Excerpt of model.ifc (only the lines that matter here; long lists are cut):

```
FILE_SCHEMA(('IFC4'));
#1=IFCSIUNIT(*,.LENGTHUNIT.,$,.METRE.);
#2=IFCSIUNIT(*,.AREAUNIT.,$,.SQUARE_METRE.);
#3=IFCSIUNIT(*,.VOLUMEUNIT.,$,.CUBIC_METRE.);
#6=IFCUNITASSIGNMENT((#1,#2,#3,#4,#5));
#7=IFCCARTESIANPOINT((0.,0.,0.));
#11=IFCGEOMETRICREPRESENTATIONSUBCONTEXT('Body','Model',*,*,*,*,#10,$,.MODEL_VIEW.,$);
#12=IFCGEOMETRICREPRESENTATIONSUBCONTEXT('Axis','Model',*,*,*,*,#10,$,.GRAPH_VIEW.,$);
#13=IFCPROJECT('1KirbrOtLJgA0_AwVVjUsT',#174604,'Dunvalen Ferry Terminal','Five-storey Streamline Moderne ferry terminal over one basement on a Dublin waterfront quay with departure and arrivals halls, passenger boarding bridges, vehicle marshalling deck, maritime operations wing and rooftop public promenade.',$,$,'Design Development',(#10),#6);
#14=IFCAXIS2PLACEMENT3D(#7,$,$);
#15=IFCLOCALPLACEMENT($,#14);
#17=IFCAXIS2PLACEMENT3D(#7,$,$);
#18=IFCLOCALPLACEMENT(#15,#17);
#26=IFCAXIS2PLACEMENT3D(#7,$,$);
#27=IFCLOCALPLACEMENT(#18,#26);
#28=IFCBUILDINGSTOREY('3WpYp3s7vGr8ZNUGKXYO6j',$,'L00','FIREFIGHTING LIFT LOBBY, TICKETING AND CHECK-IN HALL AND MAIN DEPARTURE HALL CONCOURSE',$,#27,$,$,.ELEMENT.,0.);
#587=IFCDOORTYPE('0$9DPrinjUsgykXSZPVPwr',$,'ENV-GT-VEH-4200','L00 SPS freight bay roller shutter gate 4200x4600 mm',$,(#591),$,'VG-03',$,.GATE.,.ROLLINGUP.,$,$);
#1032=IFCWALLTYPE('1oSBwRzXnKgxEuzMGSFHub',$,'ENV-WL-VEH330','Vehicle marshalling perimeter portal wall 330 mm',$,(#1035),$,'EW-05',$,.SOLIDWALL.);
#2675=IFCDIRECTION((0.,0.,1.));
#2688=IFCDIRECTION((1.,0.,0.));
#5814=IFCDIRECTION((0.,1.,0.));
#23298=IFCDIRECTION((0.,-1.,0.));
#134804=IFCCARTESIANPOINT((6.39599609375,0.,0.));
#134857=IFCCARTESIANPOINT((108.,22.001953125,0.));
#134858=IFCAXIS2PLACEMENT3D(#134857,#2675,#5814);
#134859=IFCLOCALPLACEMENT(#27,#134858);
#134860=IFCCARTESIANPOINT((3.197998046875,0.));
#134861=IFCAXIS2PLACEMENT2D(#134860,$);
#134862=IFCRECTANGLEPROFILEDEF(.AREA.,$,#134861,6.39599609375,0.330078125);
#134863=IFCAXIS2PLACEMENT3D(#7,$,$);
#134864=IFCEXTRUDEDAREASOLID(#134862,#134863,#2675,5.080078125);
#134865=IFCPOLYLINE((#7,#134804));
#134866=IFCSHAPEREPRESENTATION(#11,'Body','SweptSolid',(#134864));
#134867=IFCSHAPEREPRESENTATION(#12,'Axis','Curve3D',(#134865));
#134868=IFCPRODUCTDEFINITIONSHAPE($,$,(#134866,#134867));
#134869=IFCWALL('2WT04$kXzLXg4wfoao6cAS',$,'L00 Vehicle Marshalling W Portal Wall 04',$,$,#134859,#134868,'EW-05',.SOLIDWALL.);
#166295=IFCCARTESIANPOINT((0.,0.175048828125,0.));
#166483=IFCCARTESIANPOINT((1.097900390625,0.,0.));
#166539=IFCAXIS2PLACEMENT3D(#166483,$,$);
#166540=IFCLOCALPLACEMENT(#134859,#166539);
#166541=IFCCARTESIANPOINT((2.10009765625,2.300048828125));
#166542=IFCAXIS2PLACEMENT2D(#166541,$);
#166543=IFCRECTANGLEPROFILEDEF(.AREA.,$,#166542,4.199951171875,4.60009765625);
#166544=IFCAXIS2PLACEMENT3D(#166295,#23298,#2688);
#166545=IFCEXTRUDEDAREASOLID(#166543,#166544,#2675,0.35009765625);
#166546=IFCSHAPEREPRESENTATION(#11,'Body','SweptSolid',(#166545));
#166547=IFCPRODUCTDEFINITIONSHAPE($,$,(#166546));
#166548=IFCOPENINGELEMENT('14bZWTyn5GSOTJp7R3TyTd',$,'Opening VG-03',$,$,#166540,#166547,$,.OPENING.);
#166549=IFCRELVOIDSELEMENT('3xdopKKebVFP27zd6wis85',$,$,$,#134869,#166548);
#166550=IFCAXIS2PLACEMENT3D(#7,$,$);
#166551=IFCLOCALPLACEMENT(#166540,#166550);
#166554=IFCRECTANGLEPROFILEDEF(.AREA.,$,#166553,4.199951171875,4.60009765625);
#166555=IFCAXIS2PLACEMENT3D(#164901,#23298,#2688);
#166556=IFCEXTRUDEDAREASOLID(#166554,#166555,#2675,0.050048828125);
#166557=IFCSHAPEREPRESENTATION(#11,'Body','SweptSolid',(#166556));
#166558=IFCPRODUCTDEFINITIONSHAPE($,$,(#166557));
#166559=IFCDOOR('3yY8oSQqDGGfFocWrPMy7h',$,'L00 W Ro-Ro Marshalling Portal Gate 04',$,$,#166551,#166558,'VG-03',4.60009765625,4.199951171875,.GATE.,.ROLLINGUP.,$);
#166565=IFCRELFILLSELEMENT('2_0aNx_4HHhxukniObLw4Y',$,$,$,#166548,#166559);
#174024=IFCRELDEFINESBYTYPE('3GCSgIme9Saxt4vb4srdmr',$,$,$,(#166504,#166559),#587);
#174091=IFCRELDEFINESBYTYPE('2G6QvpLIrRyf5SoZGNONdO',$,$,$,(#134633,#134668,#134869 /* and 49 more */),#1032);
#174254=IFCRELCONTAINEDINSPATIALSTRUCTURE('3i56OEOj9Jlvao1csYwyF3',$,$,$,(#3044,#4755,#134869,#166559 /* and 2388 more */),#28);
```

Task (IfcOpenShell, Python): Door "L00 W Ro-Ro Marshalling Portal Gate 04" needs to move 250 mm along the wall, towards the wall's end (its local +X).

```python
import ifcopenshell
import ifcopenshell.api.geometry
import ifcopenshell.util.placement

model = ifcopenshell.open("model.ifc")

door = model.by_guid("3yY8oSQqDGGfFocWrPMy7h")
opening = door.FillsVoids[0].RelatingOpeningElement
wall = opening.VoidsElements[0].RelatingBuildingElement

wall_matrix = ifcopenshell.util.placement.get_local_placement(wall.ObjectPlacement)
shift = wall_matrix[:3, 0] * 0.25
before = ifcopenshell.util.placement.get_local_placement(door.ObjectPlacement)[:3, 3].copy()

# The door is placed relative to its opening, so it follows when the opening moves.
matrix = ifcopenshell.util.placement.get_local_placement(opening.ObjectPlacement)
matrix[:3, 3] += shift
ifcopenshell.api.geometry.edit_object_placement(
    model, product=opening, matrix=matrix, is_si=False, should_transform_children=True
)

after = ifcopenshell.util.placement.get_local_placement(door.ObjectPlacement)[:3, 3]
print("door moved by", (after - before).round(3) + 0.0)

model.write("model_rev.ifc")
```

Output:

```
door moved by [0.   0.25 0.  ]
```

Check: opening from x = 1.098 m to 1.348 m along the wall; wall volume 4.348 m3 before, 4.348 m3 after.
